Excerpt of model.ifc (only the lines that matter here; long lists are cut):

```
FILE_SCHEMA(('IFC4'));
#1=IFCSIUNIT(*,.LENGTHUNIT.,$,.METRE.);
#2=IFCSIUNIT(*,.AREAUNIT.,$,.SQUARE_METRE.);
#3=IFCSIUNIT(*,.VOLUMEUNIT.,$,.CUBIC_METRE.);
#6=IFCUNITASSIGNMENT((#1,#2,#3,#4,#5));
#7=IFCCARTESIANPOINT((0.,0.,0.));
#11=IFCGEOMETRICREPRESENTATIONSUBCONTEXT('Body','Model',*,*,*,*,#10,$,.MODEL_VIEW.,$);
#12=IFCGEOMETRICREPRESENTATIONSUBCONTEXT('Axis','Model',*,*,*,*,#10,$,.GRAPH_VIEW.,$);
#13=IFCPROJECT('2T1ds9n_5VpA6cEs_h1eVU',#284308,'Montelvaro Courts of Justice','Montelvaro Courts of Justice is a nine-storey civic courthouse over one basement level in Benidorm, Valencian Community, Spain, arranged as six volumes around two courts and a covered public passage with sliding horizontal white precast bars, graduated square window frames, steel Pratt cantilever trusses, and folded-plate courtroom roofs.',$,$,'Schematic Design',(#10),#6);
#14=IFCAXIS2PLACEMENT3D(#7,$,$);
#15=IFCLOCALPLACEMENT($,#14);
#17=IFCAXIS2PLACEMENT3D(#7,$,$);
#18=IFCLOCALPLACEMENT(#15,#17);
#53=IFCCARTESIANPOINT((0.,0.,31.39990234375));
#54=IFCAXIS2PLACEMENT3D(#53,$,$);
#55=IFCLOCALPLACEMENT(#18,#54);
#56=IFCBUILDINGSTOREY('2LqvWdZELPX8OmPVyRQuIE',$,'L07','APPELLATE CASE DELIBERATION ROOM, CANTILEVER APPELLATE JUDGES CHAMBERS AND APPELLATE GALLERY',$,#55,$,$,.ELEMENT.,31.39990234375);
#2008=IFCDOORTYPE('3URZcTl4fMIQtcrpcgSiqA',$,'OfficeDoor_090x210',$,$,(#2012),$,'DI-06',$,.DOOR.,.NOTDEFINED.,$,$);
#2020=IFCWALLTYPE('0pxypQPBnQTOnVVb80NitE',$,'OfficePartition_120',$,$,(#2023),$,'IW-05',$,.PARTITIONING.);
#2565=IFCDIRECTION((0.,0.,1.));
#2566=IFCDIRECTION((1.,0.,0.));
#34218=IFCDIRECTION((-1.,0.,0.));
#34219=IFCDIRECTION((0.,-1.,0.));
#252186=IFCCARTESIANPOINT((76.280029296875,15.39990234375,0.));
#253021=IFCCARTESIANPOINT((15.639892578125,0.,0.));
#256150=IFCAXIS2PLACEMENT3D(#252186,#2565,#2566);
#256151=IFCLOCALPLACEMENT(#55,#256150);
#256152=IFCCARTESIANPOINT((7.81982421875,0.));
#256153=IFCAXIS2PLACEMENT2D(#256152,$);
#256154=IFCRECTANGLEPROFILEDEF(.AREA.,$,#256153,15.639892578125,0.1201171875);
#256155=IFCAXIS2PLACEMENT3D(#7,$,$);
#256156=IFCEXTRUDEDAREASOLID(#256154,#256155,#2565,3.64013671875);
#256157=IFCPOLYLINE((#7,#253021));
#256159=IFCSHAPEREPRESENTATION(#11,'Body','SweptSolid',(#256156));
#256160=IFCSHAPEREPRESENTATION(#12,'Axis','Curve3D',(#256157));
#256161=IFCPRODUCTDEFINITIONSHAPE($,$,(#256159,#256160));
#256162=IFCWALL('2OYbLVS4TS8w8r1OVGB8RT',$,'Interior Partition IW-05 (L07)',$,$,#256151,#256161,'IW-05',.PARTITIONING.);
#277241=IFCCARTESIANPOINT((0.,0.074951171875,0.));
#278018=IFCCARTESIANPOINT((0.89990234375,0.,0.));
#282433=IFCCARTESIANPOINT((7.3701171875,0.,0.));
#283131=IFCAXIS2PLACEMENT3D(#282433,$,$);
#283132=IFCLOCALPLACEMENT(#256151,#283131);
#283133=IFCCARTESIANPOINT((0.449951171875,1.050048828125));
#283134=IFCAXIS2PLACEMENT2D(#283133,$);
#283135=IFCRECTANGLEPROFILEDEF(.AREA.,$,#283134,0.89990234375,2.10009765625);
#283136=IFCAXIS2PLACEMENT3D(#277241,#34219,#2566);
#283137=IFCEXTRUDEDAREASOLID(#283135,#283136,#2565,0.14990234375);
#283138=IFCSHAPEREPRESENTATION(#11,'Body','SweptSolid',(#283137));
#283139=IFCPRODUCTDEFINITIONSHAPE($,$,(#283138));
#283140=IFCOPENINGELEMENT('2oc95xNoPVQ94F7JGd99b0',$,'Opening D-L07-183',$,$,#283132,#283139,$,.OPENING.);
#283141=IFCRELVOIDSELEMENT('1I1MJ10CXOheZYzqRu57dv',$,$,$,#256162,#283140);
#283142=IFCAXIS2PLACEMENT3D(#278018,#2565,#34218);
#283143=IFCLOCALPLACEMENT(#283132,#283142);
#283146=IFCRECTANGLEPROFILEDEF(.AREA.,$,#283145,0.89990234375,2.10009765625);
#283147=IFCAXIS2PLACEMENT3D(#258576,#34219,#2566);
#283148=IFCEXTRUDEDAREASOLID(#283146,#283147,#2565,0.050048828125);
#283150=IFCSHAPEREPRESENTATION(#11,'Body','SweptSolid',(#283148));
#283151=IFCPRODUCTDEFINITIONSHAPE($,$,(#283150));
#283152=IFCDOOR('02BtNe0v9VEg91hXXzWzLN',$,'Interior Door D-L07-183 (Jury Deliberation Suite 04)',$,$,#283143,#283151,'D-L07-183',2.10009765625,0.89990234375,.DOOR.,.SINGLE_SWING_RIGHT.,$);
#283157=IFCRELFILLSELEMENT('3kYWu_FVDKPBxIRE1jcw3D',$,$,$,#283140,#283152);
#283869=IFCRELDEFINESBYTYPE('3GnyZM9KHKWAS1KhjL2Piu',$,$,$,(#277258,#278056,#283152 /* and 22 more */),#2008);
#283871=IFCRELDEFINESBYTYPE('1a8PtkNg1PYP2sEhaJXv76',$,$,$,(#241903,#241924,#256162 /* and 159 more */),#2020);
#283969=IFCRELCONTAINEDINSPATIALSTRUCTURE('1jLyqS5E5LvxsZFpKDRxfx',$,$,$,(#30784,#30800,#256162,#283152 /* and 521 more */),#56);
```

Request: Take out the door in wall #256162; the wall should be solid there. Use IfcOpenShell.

```python
import ifcopenshell
import ifcopenshell.api.feature
import ifcopenshell.api.root
import ifcopenshell.geom
import ifcopenshell.util.shape

model = ifcopenshell.open("model.ifc")
settings = ifcopenshell.geom.settings()


def volume(element):
    """Net volume in cubic metres, openings subtracted."""
    shape = ifcopenshell.geom.create_shape(settings, element)
    return ifcopenshell.util.shape.get_volume(shape.geometry)


door = model.by_guid("02BtNe0v9VEg91hXXzWzLN")
opening = door.FillsVoids[0].RelatingOpeningElement
wall = opening.VoidsElements[0].RelatingBuildingElement
before = volume(wall)

ifcopenshell.api.root.remove_product(model, product=door)
ifcopenshell.api.feature.remove_feature(model, feature=opening)

after = volume(wall)

print(f"wall volume {before:.3f} -> {after:.3f} m3")

model.write("model_updated.ifc")
```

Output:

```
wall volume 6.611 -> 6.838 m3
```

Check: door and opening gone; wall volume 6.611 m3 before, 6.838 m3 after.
